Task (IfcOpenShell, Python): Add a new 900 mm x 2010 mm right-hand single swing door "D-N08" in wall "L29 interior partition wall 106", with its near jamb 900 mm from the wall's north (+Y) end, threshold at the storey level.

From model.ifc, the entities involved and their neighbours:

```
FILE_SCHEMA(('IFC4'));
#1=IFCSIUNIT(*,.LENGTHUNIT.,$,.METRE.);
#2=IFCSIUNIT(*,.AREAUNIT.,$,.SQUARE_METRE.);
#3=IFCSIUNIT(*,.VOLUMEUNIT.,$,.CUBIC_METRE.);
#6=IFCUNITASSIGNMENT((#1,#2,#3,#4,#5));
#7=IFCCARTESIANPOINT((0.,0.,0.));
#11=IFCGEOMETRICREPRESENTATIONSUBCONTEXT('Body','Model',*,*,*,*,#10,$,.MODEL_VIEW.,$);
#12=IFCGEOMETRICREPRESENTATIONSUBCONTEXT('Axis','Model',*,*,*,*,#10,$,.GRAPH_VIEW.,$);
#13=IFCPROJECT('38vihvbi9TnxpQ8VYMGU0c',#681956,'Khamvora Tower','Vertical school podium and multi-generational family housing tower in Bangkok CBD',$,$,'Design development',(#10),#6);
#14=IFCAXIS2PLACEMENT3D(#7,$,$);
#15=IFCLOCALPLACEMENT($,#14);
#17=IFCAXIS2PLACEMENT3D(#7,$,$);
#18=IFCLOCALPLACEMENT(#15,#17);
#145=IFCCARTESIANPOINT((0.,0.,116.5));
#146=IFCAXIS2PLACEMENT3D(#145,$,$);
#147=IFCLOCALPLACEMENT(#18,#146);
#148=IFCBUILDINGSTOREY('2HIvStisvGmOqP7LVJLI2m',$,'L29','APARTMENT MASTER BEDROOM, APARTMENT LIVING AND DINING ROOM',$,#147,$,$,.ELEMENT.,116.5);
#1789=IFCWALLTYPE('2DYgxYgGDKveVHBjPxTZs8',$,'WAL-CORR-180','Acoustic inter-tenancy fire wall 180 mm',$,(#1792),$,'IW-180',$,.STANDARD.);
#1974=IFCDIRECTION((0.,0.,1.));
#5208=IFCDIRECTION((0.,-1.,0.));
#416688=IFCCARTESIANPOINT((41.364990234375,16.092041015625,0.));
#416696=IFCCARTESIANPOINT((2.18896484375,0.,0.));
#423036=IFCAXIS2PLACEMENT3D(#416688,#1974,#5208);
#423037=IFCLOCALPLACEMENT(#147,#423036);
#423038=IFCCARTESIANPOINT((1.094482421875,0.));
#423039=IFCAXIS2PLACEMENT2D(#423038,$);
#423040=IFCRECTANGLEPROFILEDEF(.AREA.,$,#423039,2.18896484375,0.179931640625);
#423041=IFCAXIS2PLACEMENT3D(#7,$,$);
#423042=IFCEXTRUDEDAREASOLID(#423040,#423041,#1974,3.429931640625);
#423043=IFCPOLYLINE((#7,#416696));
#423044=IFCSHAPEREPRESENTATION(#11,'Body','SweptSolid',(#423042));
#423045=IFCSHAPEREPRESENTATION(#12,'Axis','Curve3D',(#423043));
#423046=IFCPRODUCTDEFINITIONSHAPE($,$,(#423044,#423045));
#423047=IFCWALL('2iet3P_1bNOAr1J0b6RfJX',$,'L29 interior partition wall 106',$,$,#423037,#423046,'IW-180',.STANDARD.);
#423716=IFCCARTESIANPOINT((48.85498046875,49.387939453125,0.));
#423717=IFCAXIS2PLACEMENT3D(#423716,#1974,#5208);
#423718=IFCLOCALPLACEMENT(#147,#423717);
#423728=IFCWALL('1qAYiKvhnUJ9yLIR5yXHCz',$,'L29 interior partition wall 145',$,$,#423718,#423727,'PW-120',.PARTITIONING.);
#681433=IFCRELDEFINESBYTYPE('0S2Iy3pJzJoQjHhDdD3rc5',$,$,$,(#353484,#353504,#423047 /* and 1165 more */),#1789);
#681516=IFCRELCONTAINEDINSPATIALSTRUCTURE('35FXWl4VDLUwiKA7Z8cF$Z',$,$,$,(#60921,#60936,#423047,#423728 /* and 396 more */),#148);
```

```python
import numpy as np
import ifcopenshell
import ifcopenshell.api.feature
import ifcopenshell.api.geometry
import ifcopenshell.api.root
import ifcopenshell.api.spatial
import ifcopenshell.geom
import ifcopenshell.util.element
import ifcopenshell.util.placement
import ifcopenshell.util.representation
import ifcopenshell.util.shape
import ifcopenshell.util.unit

model = ifcopenshell.open("model.ifc")
unit_scale = ifcopenshell.util.unit.calculate_unit_scale(model)
settings = ifcopenshell.geom.settings()


def volume(element):
    """Net volume in cubic metres, openings subtracted."""
    shape = ifcopenshell.geom.create_shape(settings, element)
    return ifcopenshell.util.shape.get_volume(shape.geometry)


wall = model.by_guid("2iet3P_1bNOAr1J0b6RfJX")
storey = ifcopenshell.util.element.get_container(wall, ifc_class="IfcBuildingStorey")
context = ifcopenshell.util.representation.get_context(model, "Model", "Body", "MODEL_VIEW")
before = volume(wall)

width, height, from_end, sill = 0.9, 2.01, 0.9, 0.0  # metres

# The wall runs along its own X axis, and the end named is its -X end.
wall_shape = ifcopenshell.geom.create_shape(settings, wall)
x, y, z = ifcopenshell.util.shape.get_vertices(wall_shape.geometry).T
start = x.min() + from_end
face, thickness = float(y.min()), float(y.max() - y.min())
wall_matrix = ifcopenshell.util.placement.get_local_placement(wall.ObjectPlacement)
level = ifcopenshell.util.placement.get_local_placement(storey.ObjectPlacement)[2, 3]


def in_wall(x, y):
    """Placement at x, y metres in the wall's axes, at sill height."""
    matrix = wall_matrix.copy()
    matrix[:, 3] = wall_matrix @ np.array([x / unit_scale, y / unit_scale, 0.0, 1.0])
    matrix[2, 3] = level + sill / unit_scale
    return matrix


# Opening: a box that overshoots both wall faces by 50 mm.
opening = ifcopenshell.api.root.create_entity(model, ifc_class="IfcOpeningElement", predefined_type="OPENING")
box = ifcopenshell.api.geometry.add_wall_representation(
    model, context=context, length=width, height=height, thickness=thickness + 0.1
)
ifcopenshell.api.geometry.assign_representation(model, product=opening, representation=box)
ifcopenshell.api.geometry.edit_object_placement(model, product=opening, matrix=in_wall(start, face - 0.05), is_si=False)
ifcopenshell.api.feature.add_feature(model, feature=opening, element=wall)

door = ifcopenshell.api.root.create_entity(model, ifc_class="IfcDoor", name="D-N08", predefined_type="DOOR")
door.OverallWidth, door.OverallHeight = width / unit_scale, height / unit_scale
door.OperationType = "SINGLE_SWING_RIGHT"
body = ifcopenshell.api.geometry.add_door_representation(
    model,
    context=context,
    overall_width=door.OverallWidth,
    overall_height=door.OverallHeight,
    operation_type="SINGLE_SWING_RIGHT",
    lining_properties={"LiningDepth": thickness / unit_scale, "ThresholdDepth": thickness / unit_scale},
)
ifcopenshell.api.geometry.assign_representation(model, product=door, representation=body)
ifcopenshell.api.spatial.assign_container(model, products=[door], relating_structure=storey)
ifcopenshell.api.feature.add_filling(model, opening=opening, element=door)

# The lining spans the wall, so the door starts at the wall face.
ifcopenshell.api.geometry.edit_object_placement(model, product=door, matrix=in_wall(start, face), is_si=False)

after = volume(wall)

print(f"wall volume {before:.3f} -> {after:.3f} m3")

model.write("model_updated.ifc")
```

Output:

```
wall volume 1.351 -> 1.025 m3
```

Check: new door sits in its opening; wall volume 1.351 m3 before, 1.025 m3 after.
